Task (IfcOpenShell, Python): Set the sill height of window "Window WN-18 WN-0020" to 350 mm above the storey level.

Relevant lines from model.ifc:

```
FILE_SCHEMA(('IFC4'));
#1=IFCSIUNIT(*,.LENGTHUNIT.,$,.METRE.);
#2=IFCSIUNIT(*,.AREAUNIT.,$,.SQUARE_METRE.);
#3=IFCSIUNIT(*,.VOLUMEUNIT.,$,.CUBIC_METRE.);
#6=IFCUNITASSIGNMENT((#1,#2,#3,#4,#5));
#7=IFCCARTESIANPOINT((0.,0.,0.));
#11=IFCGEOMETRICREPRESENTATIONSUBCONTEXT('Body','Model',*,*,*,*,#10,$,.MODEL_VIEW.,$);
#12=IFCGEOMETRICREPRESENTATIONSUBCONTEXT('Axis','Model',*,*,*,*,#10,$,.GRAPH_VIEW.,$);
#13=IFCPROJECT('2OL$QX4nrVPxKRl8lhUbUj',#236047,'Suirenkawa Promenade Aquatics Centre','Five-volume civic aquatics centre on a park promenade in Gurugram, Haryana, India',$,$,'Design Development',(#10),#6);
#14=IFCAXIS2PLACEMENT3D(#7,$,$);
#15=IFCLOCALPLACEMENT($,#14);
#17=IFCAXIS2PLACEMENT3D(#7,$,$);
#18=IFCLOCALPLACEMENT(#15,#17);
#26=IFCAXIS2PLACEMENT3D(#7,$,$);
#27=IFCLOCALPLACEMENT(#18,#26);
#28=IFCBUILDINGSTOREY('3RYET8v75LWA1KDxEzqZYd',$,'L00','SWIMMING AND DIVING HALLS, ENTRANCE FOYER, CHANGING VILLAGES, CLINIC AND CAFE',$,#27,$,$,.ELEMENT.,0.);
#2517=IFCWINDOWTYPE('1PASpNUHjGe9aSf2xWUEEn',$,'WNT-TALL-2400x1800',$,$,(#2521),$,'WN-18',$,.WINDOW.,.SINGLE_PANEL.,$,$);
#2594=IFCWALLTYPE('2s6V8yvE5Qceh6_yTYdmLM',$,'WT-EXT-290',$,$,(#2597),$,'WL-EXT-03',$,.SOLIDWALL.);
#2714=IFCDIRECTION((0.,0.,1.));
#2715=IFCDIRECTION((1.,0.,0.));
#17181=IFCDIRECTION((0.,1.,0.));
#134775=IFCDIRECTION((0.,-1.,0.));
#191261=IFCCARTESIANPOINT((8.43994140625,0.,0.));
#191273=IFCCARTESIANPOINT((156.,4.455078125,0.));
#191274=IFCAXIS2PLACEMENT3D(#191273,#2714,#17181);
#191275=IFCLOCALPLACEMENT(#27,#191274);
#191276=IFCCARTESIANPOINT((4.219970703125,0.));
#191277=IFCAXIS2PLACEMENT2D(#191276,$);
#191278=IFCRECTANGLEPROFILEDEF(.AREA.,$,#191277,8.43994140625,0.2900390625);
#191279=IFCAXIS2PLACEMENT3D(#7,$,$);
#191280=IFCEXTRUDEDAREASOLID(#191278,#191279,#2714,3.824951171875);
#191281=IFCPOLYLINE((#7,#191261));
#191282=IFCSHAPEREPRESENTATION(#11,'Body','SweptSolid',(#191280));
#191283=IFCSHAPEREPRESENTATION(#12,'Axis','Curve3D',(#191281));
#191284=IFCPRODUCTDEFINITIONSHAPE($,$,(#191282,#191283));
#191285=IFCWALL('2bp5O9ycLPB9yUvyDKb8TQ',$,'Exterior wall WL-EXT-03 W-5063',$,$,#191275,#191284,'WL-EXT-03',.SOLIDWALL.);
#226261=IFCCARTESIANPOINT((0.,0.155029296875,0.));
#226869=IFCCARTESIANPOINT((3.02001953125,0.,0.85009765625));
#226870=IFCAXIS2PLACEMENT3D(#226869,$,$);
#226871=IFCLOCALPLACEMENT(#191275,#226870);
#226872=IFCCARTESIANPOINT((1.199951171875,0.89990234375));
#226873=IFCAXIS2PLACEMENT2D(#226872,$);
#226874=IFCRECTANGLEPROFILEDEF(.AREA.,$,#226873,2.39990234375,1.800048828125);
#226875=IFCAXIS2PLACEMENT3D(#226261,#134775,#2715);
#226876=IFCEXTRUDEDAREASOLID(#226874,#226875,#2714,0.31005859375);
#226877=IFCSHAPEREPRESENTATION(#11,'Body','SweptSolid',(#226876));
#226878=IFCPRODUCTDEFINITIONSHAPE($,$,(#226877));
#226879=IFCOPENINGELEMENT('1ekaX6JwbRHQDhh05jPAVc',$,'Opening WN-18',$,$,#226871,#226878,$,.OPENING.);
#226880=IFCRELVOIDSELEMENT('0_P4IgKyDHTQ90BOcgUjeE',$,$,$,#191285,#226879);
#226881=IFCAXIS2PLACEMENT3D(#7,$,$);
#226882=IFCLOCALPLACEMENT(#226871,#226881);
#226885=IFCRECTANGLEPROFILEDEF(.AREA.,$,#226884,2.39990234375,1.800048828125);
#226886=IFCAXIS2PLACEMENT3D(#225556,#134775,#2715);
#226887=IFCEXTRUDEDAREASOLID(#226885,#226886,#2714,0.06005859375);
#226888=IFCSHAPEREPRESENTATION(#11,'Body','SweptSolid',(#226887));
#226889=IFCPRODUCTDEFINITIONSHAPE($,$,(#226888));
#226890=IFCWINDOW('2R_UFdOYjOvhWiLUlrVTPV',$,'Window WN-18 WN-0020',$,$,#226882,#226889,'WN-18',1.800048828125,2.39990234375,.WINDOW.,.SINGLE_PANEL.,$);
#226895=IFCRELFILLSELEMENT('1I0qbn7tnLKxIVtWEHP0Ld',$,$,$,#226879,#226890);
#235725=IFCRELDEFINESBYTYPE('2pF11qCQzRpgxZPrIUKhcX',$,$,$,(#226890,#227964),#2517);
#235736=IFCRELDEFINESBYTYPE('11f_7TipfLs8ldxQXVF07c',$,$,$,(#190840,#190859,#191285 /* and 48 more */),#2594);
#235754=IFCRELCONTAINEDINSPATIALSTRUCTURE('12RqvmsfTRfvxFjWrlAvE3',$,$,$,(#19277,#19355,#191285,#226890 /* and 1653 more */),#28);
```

```python
import numpy as np
import ifcopenshell
import ifcopenshell.api.geometry
import ifcopenshell.geom
import ifcopenshell.util.element
import ifcopenshell.util.placement
import ifcopenshell.util.shape
import ifcopenshell.util.unit

model = ifcopenshell.open("model.ifc")
unit_scale = ifcopenshell.util.unit.calculate_unit_scale(model)

window = model.by_guid("2R_UFdOYjOvhWiLUlrVTPV")
opening = window.FillsVoids[0].RelatingOpeningElement
storey = ifcopenshell.util.element.get_container(window, ifc_class="IfcBuildingStorey")
level = ifcopenshell.util.placement.get_local_placement(storey.ObjectPlacement)[2, 3]

# The opening's origin need not be at the sill, so measure its lowest point.
shape = ifcopenshell.geom.create_shape(ifcopenshell.geom.settings(), opening)
bottom = ifcopenshell.util.shape.get_shape_bottom_elevation(shape, shape.geometry) / unit_scale
dz = level + 0.35 - bottom

shift = np.array([0.0, 0.0, dz])
# The window is placed relative to its opening, so it follows when the opening moves.
matrix = ifcopenshell.util.placement.get_local_placement(opening.ObjectPlacement)
matrix[:3, 3] += shift
ifcopenshell.api.geometry.edit_object_placement(
    model, product=opening, matrix=matrix, is_si=False, should_transform_children=True
)

print(f"moved by {dz * unit_scale:+.3f} m")

model.write("model_updated.ifc")
```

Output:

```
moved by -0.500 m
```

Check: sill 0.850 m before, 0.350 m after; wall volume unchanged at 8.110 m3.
